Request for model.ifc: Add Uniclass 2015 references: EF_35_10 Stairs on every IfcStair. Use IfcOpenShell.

First a look at what the model holds.

```python
import ifcopenshell

model = ifcopenshell.open("model.ifc")
print(model.schema)
print("classifications:", [c.Name for c in model.by_type("IfcClassification")])
for ifc_class in ("IfcDoor", "IfcRoof", "IfcStair", "IfcWall", "IfcWindow"):
    print(ifc_class, len(model.by_type(ifc_class)))
```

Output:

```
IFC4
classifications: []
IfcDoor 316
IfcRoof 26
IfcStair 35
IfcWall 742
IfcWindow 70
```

```python
import ifcopenshell
import ifcopenshell.api.classification

model = ifcopenshell.open("model.ifc")

system = ifcopenshell.api.classification.add_classification(model, classification="Uniclass 2015")

codes = {
    "IfcStair": ("EF_35_10", "Stairs"),
}
for ifc_class, (code, name) in codes.items():
    products = model.by_type(ifc_class)
    ifcopenshell.api.classification.add_reference(
        model, products=products, classification=system, identification=code, name=name
    )
    print(code, len(products))

model.write("model-out.ifc")
```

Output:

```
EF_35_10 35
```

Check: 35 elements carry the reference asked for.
